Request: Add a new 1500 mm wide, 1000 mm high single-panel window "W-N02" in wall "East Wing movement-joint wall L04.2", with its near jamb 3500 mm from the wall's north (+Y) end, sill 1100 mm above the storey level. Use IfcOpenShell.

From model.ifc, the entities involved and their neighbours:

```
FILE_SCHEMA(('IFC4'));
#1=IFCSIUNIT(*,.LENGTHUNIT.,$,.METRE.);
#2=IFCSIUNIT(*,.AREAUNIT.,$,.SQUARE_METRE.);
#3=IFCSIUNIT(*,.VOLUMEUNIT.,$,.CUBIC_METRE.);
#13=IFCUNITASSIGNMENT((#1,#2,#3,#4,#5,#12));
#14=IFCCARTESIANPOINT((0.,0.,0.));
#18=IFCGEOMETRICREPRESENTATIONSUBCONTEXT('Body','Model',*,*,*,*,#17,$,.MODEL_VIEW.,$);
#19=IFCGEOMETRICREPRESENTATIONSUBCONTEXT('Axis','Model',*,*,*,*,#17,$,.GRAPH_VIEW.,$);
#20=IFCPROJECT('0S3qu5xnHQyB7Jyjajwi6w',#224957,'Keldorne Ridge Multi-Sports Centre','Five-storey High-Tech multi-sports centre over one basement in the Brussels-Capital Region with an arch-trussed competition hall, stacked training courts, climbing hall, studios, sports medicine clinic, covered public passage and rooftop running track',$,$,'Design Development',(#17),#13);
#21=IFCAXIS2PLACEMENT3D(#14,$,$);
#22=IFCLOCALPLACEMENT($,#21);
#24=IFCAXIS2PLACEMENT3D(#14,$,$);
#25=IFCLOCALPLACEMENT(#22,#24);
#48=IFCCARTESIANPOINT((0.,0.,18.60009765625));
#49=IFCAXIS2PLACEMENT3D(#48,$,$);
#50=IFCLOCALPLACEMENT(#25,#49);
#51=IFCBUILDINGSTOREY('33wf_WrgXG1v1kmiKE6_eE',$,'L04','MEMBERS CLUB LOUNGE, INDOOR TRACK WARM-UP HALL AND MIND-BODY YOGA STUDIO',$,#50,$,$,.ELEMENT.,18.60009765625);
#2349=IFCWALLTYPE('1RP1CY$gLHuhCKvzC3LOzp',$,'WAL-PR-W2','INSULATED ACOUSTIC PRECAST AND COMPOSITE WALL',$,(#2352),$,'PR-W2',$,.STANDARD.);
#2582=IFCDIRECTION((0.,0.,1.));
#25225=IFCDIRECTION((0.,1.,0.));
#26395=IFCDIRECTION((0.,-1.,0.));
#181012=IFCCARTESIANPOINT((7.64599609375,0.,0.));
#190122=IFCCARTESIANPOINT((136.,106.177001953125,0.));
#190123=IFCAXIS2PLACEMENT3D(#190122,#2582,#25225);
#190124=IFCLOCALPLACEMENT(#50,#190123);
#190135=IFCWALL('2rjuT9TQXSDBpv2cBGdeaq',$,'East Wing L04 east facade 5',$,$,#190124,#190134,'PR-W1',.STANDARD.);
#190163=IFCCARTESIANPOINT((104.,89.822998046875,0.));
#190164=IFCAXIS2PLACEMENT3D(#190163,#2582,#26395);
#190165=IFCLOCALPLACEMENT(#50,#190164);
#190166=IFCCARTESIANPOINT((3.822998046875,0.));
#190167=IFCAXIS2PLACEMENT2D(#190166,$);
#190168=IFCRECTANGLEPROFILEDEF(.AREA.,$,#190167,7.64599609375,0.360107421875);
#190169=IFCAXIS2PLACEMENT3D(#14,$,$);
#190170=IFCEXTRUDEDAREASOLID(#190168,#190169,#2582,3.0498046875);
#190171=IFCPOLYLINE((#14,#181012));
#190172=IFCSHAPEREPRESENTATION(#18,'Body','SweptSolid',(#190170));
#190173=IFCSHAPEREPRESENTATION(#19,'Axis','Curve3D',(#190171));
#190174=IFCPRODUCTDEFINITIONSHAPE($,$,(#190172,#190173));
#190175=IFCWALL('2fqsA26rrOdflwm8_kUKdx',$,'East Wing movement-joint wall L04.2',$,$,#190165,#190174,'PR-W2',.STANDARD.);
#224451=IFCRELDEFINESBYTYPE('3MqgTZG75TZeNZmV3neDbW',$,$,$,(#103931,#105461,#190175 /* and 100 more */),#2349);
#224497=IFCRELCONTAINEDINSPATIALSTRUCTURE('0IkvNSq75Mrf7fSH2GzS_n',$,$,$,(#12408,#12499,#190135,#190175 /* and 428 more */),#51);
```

```python
import numpy as np
import ifcopenshell
import ifcopenshell.api.feature
import ifcopenshell.api.geometry
import ifcopenshell.api.root
import ifcopenshell.api.spatial
import ifcopenshell.geom
import ifcopenshell.util.element
import ifcopenshell.util.placement
import ifcopenshell.util.representation
import ifcopenshell.util.shape
import ifcopenshell.util.unit

model = ifcopenshell.open("model.ifc")
unit_scale = ifcopenshell.util.unit.calculate_unit_scale(model)
settings = ifcopenshell.geom.settings()


def volume(element):
    """Net volume in cubic metres, openings subtracted."""
    shape = ifcopenshell.geom.create_shape(settings, element)
    return ifcopenshell.util.shape.get_volume(shape.geometry)


wall = model.by_guid("2fqsA26rrOdflwm8_kUKdx")
storey = ifcopenshell.util.element.get_container(wall, ifc_class="IfcBuildingStorey")
context = ifcopenshell.util.representation.get_context(model, "Model", "Body", "MODEL_VIEW")
before = volume(wall)

width, height, from_end, sill = 1.5, 1, 3.5, 1.1  # metres

# The wall runs along its own X axis, and the end named is its -X end.
wall_shape = ifcopenshell.geom.create_shape(settings, wall)
x, y, z = ifcopenshell.util.shape.get_vertices(wall_shape.geometry).T
start = x.min() + from_end
face, thickness = float(y.min()), float(y.max() - y.min())
wall_matrix = ifcopenshell.util.placement.get_local_placement(wall.ObjectPlacement)
level = ifcopenshell.util.placement.get_local_placement(storey.ObjectPlacement)[2, 3]


def in_wall(x, y):
    """Placement at x, y metres in the wall's axes, at sill height."""
    matrix = wall_matrix.copy()
    matrix[:, 3] = wall_matrix @ np.array([x / unit_scale, y / unit_scale, 0.0, 1.0])
    matrix[2, 3] = level + sill / unit_scale
    return matrix


# Opening: a box that overshoots both wall faces by 50 mm.
opening = ifcopenshell.api.root.create_entity(model, ifc_class="IfcOpeningElement", predefined_type="OPENING")
box = ifcopenshell.api.geometry.add_wall_representation(
    model, context=context, length=width, height=height, thickness=thickness + 0.1
)
ifcopenshell.api.geometry.assign_representation(model, product=opening, representation=box)
ifcopenshell.api.geometry.edit_object_placement(model, product=opening, matrix=in_wall(start, face - 0.05), is_si=False)
ifcopenshell.api.feature.add_feature(model, feature=opening, element=wall)

window = ifcopenshell.api.root.create_entity(model, ifc_class="IfcWindow", name="W-N02", predefined_type="WINDOW")
window.OverallWidth, window.OverallHeight = width / unit_scale, height / unit_scale
window.PartitioningType = "SINGLE_PANEL"
body = ifcopenshell.api.geometry.add_window_representation(
    model,
    context=context,
    overall_width=window.OverallWidth,
    overall_height=window.OverallHeight,
    partition_type="SINGLE_PANEL",
)
ifcopenshell.api.geometry.assign_representation(model, product=window, representation=body)
ifcopenshell.api.spatial.assign_container(model, products=[window], relating_structure=storey)
ifcopenshell.api.feature.add_filling(model, opening=opening, element=window)

# Centre the window in the wall's thickness.
ifcopenshell.api.geometry.edit_object_placement(model, product=window, matrix=in_wall(start, face), is_si=False)
window_shape = ifcopenshell.geom.create_shape(settings, window)
depth = ifcopenshell.util.shape.get_vertices(window_shape.geometry)[:, 1]
offset = face + thickness / 2 - (depth.min() + depth.max()) / 2
ifcopenshell.api.geometry.edit_object_placement(model, product=window, matrix=in_wall(start, offset), is_si=False)

after = volume(wall)

print(f"wall volume {before:.3f} -> {after:.3f} m3")

model.write("model_v2.ifc")
```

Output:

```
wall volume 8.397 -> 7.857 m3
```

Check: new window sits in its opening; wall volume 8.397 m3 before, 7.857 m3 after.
